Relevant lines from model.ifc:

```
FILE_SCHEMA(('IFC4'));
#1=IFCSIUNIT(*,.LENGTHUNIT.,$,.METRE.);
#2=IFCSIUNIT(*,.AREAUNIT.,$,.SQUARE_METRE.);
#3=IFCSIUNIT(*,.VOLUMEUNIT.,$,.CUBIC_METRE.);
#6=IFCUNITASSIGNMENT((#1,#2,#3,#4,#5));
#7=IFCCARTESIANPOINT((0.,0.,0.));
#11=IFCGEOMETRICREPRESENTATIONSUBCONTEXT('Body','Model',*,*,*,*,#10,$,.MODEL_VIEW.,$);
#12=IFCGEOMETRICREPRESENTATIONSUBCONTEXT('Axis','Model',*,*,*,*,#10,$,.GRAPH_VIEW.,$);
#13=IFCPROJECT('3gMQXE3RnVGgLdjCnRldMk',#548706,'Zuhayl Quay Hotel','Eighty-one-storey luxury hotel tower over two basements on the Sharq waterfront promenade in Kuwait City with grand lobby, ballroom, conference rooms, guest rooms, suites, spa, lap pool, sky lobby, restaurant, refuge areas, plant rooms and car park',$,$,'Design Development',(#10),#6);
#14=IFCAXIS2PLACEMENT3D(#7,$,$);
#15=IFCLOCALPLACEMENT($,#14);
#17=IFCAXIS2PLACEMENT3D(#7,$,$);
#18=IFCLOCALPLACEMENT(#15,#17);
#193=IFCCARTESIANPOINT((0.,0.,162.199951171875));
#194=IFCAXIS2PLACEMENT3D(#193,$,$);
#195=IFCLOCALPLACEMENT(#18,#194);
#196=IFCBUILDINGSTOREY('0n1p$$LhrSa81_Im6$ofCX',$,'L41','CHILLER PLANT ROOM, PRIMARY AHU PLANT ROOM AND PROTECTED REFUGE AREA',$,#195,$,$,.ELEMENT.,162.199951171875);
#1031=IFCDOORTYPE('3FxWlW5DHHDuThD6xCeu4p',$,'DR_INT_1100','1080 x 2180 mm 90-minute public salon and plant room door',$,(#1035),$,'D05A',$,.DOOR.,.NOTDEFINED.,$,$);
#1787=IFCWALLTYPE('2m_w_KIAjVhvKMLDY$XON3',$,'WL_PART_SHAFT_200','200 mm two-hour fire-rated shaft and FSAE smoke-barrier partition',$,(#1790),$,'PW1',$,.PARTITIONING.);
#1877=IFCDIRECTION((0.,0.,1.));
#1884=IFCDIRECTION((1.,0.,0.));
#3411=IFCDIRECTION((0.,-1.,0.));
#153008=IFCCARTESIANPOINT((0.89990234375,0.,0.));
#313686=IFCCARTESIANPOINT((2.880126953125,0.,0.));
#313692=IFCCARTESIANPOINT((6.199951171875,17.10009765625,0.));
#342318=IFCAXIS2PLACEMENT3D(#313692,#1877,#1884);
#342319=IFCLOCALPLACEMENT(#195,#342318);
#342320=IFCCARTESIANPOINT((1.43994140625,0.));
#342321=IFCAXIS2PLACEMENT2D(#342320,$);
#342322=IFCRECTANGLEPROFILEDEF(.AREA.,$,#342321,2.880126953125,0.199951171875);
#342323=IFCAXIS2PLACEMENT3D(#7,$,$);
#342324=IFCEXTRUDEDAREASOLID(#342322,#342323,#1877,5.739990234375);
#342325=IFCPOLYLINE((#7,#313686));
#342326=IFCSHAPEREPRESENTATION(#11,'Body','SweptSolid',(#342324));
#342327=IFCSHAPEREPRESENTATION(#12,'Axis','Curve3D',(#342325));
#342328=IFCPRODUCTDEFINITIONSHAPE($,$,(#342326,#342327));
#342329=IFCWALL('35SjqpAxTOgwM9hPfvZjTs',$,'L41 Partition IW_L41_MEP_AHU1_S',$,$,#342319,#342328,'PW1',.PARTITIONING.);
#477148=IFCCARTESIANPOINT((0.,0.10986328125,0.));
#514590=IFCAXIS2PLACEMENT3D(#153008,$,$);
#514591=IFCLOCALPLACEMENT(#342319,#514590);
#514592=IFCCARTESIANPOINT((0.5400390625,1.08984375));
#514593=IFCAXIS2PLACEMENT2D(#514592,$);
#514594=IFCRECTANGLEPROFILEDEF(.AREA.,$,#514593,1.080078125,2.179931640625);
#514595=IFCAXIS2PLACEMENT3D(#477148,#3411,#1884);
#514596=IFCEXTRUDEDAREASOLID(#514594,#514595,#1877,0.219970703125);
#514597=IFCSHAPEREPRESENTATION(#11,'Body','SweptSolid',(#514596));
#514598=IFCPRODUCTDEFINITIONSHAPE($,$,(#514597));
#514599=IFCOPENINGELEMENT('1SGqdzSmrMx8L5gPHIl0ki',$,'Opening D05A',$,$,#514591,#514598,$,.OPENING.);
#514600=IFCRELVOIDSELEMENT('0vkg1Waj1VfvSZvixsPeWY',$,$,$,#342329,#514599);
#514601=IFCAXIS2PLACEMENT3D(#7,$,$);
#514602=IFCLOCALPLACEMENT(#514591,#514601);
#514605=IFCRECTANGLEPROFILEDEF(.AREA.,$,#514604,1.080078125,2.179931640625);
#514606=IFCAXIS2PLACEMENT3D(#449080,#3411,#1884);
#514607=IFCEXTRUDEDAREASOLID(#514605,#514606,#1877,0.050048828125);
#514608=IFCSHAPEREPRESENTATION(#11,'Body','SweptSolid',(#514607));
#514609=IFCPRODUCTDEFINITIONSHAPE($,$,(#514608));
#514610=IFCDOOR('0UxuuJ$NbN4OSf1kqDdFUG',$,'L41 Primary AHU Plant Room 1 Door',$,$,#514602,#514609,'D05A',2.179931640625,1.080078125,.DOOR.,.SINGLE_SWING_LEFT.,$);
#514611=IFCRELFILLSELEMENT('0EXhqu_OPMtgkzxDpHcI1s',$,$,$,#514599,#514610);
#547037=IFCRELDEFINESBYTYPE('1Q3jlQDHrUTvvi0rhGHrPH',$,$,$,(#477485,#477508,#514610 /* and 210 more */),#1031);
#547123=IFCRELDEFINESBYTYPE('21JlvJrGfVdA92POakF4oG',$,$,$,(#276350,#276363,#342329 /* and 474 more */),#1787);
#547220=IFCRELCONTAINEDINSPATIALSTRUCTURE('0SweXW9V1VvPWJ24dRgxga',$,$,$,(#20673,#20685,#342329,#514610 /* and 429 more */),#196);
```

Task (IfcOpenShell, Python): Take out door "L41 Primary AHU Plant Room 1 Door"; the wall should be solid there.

```python
import ifcopenshell
import ifcopenshell.api.feature
import ifcopenshell.api.root
import ifcopenshell.geom
import ifcopenshell.util.shape

model = ifcopenshell.open("model.ifc")
settings = ifcopenshell.geom.settings()


def volume(element):
    """Net volume in cubic metres, openings subtracted."""
    shape = ifcopenshell.geom.create_shape(settings, element)
    return ifcopenshell.util.shape.get_volume(shape.geometry)


door = model.by_guid("0UxuuJ$NbN4OSf1kqDdFUG")
opening = door.FillsVoids[0].RelatingOpeningElement
wall = opening.VoidsElements[0].RelatingBuildingElement
before = volume(wall)

ifcopenshell.api.root.remove_product(model, product=door)
ifcopenshell.api.feature.remove_feature(model, feature=opening)

after = volume(wall)

print(f"wall volume {before:.3f} -> {after:.3f} m3")

model.write("model_updated.ifc")
```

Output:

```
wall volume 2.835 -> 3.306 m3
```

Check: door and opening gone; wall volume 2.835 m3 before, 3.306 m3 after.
